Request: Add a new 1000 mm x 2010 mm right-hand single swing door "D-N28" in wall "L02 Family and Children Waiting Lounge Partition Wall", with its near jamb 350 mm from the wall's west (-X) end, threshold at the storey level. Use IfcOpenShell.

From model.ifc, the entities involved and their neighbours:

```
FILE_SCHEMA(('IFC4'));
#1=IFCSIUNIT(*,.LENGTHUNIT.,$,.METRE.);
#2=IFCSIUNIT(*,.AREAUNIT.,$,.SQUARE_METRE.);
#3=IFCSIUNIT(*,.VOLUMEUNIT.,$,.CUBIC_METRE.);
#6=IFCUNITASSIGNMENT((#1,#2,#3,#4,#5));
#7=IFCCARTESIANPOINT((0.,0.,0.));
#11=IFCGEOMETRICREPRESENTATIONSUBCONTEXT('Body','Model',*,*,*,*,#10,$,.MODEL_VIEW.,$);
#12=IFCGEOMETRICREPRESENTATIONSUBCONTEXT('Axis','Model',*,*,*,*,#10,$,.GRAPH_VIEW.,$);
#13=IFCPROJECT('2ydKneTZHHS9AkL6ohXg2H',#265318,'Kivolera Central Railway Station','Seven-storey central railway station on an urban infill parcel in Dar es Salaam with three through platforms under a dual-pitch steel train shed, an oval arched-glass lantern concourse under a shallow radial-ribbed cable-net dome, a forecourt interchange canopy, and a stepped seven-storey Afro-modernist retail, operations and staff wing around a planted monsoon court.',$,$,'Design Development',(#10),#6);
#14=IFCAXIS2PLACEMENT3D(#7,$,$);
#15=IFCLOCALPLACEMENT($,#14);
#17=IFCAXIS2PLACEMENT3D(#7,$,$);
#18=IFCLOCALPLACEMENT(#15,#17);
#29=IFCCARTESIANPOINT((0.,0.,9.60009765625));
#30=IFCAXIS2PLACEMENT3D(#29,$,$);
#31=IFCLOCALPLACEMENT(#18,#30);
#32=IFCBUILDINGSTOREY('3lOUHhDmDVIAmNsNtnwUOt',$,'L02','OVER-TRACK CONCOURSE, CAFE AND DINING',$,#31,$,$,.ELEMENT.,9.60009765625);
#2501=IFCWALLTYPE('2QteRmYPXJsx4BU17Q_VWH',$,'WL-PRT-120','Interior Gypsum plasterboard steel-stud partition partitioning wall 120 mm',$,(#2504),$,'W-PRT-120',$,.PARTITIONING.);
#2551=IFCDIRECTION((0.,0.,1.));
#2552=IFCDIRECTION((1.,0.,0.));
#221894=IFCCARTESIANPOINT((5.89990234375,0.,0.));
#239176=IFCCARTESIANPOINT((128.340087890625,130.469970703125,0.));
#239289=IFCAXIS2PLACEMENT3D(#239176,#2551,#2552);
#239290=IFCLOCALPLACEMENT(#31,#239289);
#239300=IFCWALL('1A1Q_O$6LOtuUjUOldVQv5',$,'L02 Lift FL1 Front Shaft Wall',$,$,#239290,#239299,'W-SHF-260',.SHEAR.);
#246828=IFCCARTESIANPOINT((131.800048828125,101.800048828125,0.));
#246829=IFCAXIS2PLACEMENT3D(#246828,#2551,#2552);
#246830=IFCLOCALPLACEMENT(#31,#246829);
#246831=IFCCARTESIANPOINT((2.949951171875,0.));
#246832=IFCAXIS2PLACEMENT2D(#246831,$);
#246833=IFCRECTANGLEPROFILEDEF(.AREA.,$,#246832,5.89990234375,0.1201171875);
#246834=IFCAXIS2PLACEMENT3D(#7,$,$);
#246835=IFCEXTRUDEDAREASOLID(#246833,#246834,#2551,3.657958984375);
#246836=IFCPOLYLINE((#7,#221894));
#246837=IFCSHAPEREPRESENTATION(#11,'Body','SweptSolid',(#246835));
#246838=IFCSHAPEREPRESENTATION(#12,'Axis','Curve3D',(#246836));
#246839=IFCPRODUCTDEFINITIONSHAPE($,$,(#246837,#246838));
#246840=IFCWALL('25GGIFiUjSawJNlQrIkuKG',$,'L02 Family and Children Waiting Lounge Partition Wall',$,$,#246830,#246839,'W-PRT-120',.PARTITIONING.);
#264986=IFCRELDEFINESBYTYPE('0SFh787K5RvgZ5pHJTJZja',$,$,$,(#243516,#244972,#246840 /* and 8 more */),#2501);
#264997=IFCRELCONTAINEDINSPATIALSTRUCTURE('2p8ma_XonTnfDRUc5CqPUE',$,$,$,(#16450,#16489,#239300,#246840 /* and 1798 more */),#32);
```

```python
import numpy as np
import ifcopenshell
import ifcopenshell.api.feature
import ifcopenshell.api.geometry
import ifcopenshell.api.root
import ifcopenshell.api.spatial
import ifcopenshell.geom
import ifcopenshell.util.element
import ifcopenshell.util.placement
import ifcopenshell.util.representation
import ifcopenshell.util.shape
import ifcopenshell.util.unit

model = ifcopenshell.open("model.ifc")
unit_scale = ifcopenshell.util.unit.calculate_unit_scale(model)
settings = ifcopenshell.geom.settings()


def volume(element):
    """Net volume in cubic metres, openings subtracted."""
    shape = ifcopenshell.geom.create_shape(settings, element)
    return ifcopenshell.util.shape.get_volume(shape.geometry)


wall = model.by_id(246840)
storey = ifcopenshell.util.element.get_container(wall, ifc_class="IfcBuildingStorey")
context = ifcopenshell.util.representation.get_context(model, "Model", "Body", "MODEL_VIEW")
before = volume(wall)

width, height, from_end, sill = 1, 2.01, 0.35, 0.0  # metres

# The wall runs along its own X axis, and the end named is its -X end.
wall_shape = ifcopenshell.geom.create_shape(settings, wall)
x, y, z = ifcopenshell.util.shape.get_vertices(wall_shape.geometry).T
start = x.min() + from_end
face, thickness = float(y.min()), float(y.max() - y.min())
wall_matrix = ifcopenshell.util.placement.get_local_placement(wall.ObjectPlacement)
level = ifcopenshell.util.placement.get_local_placement(storey.ObjectPlacement)[2, 3]


def in_wall(x, y):
    """Placement at x, y metres in the wall's axes, at sill height."""
    matrix = wall_matrix.copy()
    matrix[:, 3] = wall_matrix @ np.array([x / unit_scale, y / unit_scale, 0.0, 1.0])
    matrix[2, 3] = level + sill / unit_scale
    return matrix


# Opening: a box that overshoots both wall faces by 50 mm.
opening = ifcopenshell.api.root.create_entity(model, ifc_class="IfcOpeningElement", predefined_type="OPENING")
box = ifcopenshell.api.geometry.add_wall_representation(
    model, context=context, length=width, height=height, thickness=thickness + 0.1
)
ifcopenshell.api.geometry.assign_representation(model, product=opening, representation=box)
ifcopenshell.api.geometry.edit_object_placement(model, product=opening, matrix=in_wall(start, face - 0.05), is_si=False)
ifcopenshell.api.feature.add_feature(model, feature=opening, element=wall)

door = ifcopenshell.api.root.create_entity(model, ifc_class="IfcDoor", name="D-N28", predefined_type="DOOR")
door.OverallWidth, door.OverallHeight = width / unit_scale, height / unit_scale
door.OperationType = "SINGLE_SWING_RIGHT"
body = ifcopenshell.api.geometry.add_door_representation(
    model,
    context=context,
    overall_width=door.OverallWidth,
    overall_height=door.OverallHeight,
    operation_type="SINGLE_SWING_RIGHT",
    lining_properties={"LiningDepth": thickness / unit_scale, "ThresholdDepth": thickness / unit_scale},
)
ifcopenshell.api.geometry.assign_representation(model, product=door, representation=body)
ifcopenshell.api.spatial.assign_container(model, products=[door], relating_structure=storey)
ifcopenshell.api.feature.add_filling(model, opening=opening, element=door)

# The lining spans the wall, so the door starts at the wall face.
ifcopenshell.api.geometry.edit_object_placement(model, product=door, matrix=in_wall(start, face), is_si=False)

after = volume(wall)

print(f"wall volume {before:.3f} -> {after:.3f} m3")

model.write("model_v2.ifc")
```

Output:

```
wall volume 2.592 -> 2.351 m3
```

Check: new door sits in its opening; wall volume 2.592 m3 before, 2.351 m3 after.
